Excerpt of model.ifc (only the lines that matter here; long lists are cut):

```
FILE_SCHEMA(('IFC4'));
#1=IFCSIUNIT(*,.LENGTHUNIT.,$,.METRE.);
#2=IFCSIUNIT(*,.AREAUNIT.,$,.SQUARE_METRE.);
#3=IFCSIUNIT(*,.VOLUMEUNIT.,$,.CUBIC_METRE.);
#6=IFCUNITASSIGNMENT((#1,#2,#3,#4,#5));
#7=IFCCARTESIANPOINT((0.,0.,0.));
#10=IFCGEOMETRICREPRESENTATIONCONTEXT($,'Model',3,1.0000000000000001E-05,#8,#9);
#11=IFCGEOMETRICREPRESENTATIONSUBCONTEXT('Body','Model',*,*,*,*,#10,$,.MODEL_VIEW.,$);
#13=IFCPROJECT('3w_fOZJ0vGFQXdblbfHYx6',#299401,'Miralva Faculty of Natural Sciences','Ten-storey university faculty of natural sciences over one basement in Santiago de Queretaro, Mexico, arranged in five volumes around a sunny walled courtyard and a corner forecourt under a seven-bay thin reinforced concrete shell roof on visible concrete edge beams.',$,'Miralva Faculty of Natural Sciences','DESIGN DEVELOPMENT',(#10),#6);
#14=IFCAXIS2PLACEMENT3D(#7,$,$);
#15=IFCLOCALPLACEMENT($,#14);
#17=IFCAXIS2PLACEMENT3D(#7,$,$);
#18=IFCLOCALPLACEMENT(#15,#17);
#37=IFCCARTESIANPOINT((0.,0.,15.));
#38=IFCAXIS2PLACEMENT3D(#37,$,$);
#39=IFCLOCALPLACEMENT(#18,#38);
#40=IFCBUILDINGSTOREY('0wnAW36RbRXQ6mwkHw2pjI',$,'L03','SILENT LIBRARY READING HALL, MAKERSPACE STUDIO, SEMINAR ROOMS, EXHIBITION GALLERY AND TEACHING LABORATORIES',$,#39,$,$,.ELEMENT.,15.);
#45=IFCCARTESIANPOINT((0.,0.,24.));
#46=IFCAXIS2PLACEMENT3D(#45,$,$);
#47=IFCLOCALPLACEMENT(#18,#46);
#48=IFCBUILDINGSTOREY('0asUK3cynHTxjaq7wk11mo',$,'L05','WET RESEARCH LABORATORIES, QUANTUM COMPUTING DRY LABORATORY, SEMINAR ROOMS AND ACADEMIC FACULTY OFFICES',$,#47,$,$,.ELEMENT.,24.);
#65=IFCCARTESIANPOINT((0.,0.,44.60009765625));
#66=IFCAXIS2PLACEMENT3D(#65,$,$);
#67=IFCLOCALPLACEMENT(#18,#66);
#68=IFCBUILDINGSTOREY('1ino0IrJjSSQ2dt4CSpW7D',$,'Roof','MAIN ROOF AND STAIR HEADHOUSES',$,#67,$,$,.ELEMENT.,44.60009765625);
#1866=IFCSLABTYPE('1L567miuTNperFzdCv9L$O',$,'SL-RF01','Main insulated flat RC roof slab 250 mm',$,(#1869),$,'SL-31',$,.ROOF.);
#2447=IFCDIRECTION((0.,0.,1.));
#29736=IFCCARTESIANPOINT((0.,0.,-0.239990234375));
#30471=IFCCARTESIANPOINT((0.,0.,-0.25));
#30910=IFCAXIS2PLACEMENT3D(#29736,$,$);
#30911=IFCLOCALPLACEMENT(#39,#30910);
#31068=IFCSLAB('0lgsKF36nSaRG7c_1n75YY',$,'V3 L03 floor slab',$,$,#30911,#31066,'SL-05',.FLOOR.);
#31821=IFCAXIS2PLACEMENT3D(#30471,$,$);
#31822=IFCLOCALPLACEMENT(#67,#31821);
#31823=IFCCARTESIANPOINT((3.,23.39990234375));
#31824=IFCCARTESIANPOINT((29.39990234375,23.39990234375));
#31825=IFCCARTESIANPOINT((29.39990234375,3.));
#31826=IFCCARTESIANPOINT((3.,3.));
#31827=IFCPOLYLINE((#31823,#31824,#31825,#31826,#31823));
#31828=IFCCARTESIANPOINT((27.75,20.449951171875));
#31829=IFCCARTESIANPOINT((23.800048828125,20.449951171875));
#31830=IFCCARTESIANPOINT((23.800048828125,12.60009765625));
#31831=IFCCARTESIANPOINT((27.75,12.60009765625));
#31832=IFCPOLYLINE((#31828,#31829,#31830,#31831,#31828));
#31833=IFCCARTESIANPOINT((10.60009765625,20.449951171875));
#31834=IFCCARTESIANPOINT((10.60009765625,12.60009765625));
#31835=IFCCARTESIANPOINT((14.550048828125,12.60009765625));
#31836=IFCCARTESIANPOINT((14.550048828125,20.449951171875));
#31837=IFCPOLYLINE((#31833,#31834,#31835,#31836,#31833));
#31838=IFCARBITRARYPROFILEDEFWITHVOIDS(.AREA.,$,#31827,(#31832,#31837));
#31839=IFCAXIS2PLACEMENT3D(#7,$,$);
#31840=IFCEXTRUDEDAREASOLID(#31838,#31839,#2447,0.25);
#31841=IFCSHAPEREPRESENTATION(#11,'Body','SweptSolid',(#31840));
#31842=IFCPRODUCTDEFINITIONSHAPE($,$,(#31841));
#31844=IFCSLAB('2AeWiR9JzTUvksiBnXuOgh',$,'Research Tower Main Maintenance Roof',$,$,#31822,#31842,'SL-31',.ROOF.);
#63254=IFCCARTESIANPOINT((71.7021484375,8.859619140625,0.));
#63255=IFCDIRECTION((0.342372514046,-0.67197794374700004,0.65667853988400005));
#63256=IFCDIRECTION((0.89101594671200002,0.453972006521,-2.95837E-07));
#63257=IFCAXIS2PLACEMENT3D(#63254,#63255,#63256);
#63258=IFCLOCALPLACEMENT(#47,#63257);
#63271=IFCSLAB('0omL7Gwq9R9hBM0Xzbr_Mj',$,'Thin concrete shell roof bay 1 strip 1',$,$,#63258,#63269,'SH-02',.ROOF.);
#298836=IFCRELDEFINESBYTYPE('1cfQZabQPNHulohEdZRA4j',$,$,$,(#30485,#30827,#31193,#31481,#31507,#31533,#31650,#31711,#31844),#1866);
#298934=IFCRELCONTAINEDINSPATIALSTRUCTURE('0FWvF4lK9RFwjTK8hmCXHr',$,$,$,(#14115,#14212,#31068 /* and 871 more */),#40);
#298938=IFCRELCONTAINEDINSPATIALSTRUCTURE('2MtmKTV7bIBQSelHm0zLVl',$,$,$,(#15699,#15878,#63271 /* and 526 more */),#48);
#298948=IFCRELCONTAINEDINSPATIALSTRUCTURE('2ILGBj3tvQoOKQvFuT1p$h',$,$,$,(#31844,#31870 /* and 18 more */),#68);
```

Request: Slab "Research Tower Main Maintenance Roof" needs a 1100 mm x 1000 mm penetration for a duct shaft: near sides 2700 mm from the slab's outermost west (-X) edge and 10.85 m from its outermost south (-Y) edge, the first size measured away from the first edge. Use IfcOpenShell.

```python
import numpy as np
import ifcopenshell
import ifcopenshell.api.feature
import ifcopenshell.api.geometry
import ifcopenshell.api.root
import ifcopenshell.geom
import ifcopenshell.util.placement
import ifcopenshell.util.representation
import ifcopenshell.util.shape
import ifcopenshell.util.unit

model = ifcopenshell.open("model.ifc")
unit_scale = ifcopenshell.util.unit.calculate_unit_scale(model)
settings = ifcopenshell.geom.settings()


def volume(element):
    """Net volume in cubic metres, openings subtracted."""
    shape = ifcopenshell.geom.create_shape(settings, element)
    return ifcopenshell.util.shape.get_volume(shape.geometry)


slab = model.by_guid("2AeWiR9JzTUvksiBnXuOgh")
before = volume(slab)

# Extent in the slab's own axes, in metres. The edges named are its -X and -Y sides.
slab_shape = ifcopenshell.geom.create_shape(settings, slab)
vertices = ifcopenshell.util.shape.get_vertices(slab_shape.geometry)
x_min, y_min, bottom = vertices.min(axis=0)
top = vertices[:, 2].max()

opening = ifcopenshell.api.root.create_entity(model, ifc_class="IfcOpeningElement", name="Duct shaft opening", predefined_type="OPENING")
context = ifcopenshell.util.representation.get_context(model, "Model", "Body", "MODEL_VIEW")
width, depth = 1.1, 1
outline = [(0.0, 0.0), (width, 0.0), (width, depth), (0.0, depth), (0.0, 0.0)]
# Overshoot both faces by 50 mm so the cut is clean.
shape = ifcopenshell.api.geometry.add_slab_representation(
    model, context=context, depth=top - bottom + 0.1, polyline=outline
)
ifcopenshell.api.geometry.assign_representation(model, product=opening, representation=shape)

matrix = ifcopenshell.util.placement.get_local_placement(slab.ObjectPlacement)
matrix[:, 3] = matrix @ np.append(np.array([x_min + 2.7, y_min + 10.85, bottom - 0.05]) / unit_scale, 1.0)
ifcopenshell.api.geometry.edit_object_placement(model, product=opening, matrix=matrix, is_si=False)
ifcopenshell.api.feature.add_feature(model, feature=opening, element=slab)

after = volume(slab)

print(f"slab volume {before:.3f} -> {after:.3f} m3")

model.write("model_rev.ifc")
```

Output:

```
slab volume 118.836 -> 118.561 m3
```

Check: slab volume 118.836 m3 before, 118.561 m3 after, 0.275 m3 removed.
